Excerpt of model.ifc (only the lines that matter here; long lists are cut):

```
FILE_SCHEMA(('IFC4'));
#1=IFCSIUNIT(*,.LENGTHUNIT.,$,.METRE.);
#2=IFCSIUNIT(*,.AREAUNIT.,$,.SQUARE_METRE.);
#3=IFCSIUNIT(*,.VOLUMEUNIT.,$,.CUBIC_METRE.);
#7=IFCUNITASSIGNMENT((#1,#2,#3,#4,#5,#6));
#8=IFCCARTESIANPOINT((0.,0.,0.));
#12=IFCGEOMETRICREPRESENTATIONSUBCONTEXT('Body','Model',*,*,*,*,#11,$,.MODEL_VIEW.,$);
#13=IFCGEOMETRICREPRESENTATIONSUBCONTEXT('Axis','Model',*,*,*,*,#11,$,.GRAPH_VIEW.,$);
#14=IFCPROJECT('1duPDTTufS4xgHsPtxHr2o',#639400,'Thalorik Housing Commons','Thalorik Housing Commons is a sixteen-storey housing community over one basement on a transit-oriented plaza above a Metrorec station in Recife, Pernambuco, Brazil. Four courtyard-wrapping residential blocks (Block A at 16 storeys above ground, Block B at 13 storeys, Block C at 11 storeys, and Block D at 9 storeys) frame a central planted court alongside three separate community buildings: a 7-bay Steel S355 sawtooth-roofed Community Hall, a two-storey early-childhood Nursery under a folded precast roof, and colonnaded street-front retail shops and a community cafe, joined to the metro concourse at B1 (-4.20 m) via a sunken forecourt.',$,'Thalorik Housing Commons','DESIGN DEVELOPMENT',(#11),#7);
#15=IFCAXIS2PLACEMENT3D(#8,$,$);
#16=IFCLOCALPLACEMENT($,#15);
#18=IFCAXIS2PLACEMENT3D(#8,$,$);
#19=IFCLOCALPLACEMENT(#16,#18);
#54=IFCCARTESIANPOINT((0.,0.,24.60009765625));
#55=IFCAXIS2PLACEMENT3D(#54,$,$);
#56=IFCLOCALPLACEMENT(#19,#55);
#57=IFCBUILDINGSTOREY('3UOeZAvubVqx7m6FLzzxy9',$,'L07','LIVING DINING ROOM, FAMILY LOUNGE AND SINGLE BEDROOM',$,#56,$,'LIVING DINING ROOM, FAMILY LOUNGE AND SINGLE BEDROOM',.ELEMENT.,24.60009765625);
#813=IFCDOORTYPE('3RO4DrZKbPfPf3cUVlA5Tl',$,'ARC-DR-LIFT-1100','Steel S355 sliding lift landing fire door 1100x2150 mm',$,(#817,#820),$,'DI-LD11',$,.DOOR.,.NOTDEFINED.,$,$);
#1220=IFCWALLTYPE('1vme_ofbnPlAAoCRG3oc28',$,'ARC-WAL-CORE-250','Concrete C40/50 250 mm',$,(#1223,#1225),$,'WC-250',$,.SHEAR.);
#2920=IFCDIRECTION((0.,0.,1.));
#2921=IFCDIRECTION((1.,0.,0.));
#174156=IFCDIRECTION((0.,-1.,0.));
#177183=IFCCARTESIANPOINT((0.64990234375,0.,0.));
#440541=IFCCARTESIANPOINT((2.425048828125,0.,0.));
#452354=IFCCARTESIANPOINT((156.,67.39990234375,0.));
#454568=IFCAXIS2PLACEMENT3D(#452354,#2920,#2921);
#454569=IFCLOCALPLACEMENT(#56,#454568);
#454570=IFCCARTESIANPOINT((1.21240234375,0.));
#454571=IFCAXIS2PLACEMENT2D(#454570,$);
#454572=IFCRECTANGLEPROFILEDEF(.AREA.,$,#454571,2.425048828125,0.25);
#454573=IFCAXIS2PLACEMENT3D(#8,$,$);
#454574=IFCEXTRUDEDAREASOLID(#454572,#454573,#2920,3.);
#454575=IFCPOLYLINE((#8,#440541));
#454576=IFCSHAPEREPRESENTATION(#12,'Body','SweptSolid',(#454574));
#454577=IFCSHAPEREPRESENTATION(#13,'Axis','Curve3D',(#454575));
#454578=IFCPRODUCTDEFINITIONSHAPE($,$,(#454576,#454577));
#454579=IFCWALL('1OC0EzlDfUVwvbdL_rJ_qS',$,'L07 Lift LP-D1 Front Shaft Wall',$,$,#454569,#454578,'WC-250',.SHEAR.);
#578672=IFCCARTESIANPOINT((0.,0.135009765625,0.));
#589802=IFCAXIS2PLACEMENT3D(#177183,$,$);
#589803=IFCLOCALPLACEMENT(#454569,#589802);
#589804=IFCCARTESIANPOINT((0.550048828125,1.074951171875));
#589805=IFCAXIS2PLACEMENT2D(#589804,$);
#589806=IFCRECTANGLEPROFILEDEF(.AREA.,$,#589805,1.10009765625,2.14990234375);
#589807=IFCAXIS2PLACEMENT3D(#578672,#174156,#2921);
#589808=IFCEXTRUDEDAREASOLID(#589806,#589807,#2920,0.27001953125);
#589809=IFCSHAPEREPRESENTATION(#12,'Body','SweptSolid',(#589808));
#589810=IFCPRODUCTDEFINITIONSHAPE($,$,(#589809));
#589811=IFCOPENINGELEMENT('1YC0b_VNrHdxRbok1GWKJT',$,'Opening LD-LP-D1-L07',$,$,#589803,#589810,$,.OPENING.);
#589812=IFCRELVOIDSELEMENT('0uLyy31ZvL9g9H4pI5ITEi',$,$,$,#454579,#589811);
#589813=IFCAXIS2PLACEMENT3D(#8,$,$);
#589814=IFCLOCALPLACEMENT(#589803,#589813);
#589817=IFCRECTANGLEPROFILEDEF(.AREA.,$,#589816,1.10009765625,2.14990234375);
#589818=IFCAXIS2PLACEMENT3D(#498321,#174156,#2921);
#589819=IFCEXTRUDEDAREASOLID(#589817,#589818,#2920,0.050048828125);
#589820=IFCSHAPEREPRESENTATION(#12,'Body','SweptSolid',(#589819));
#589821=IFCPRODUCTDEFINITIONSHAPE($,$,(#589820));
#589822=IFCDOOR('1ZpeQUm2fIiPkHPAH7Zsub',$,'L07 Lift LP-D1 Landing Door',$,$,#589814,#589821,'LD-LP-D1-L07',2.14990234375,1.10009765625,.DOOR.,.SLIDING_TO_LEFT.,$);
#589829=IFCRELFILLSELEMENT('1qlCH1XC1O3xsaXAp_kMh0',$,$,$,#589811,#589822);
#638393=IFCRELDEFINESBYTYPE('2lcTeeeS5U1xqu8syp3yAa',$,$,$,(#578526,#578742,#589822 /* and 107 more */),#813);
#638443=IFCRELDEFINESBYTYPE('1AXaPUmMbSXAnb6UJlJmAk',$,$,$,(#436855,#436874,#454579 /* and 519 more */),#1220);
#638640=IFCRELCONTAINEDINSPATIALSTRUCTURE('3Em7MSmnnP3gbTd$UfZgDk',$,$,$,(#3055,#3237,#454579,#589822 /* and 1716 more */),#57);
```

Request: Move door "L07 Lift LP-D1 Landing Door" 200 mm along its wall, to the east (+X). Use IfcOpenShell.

```python
import ifcopenshell
import ifcopenshell.api.geometry
import ifcopenshell.util.placement
import ifcopenshell.util.unit

model = ifcopenshell.open("model.ifc")
unit_scale = ifcopenshell.util.unit.calculate_unit_scale(model)

door = model.by_guid("1ZpeQUm2fIiPkHPAH7Zsub")
opening = door.FillsVoids[0].RelatingOpeningElement
wall = opening.VoidsElements[0].RelatingBuildingElement

wall_matrix = ifcopenshell.util.placement.get_local_placement(wall.ObjectPlacement)
shift = wall_matrix[:3, 0] * 0.2 / unit_scale
before = ifcopenshell.util.placement.get_local_placement(door.ObjectPlacement)[:3, 3].copy()

# The door is placed relative to its opening, so it follows when the opening moves.
matrix = ifcopenshell.util.placement.get_local_placement(opening.ObjectPlacement)
matrix[:3, 3] += shift
ifcopenshell.api.geometry.edit_object_placement(
    model, product=opening, matrix=matrix, is_si=False, should_transform_children=True
)

after = ifcopenshell.util.placement.get_local_placement(door.ObjectPlacement)[:3, 3]
print("door moved by", (after - before).round(3) + 0.0)

model.write("model_updated.ifc")
```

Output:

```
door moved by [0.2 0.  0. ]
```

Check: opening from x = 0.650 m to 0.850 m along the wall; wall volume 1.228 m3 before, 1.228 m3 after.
